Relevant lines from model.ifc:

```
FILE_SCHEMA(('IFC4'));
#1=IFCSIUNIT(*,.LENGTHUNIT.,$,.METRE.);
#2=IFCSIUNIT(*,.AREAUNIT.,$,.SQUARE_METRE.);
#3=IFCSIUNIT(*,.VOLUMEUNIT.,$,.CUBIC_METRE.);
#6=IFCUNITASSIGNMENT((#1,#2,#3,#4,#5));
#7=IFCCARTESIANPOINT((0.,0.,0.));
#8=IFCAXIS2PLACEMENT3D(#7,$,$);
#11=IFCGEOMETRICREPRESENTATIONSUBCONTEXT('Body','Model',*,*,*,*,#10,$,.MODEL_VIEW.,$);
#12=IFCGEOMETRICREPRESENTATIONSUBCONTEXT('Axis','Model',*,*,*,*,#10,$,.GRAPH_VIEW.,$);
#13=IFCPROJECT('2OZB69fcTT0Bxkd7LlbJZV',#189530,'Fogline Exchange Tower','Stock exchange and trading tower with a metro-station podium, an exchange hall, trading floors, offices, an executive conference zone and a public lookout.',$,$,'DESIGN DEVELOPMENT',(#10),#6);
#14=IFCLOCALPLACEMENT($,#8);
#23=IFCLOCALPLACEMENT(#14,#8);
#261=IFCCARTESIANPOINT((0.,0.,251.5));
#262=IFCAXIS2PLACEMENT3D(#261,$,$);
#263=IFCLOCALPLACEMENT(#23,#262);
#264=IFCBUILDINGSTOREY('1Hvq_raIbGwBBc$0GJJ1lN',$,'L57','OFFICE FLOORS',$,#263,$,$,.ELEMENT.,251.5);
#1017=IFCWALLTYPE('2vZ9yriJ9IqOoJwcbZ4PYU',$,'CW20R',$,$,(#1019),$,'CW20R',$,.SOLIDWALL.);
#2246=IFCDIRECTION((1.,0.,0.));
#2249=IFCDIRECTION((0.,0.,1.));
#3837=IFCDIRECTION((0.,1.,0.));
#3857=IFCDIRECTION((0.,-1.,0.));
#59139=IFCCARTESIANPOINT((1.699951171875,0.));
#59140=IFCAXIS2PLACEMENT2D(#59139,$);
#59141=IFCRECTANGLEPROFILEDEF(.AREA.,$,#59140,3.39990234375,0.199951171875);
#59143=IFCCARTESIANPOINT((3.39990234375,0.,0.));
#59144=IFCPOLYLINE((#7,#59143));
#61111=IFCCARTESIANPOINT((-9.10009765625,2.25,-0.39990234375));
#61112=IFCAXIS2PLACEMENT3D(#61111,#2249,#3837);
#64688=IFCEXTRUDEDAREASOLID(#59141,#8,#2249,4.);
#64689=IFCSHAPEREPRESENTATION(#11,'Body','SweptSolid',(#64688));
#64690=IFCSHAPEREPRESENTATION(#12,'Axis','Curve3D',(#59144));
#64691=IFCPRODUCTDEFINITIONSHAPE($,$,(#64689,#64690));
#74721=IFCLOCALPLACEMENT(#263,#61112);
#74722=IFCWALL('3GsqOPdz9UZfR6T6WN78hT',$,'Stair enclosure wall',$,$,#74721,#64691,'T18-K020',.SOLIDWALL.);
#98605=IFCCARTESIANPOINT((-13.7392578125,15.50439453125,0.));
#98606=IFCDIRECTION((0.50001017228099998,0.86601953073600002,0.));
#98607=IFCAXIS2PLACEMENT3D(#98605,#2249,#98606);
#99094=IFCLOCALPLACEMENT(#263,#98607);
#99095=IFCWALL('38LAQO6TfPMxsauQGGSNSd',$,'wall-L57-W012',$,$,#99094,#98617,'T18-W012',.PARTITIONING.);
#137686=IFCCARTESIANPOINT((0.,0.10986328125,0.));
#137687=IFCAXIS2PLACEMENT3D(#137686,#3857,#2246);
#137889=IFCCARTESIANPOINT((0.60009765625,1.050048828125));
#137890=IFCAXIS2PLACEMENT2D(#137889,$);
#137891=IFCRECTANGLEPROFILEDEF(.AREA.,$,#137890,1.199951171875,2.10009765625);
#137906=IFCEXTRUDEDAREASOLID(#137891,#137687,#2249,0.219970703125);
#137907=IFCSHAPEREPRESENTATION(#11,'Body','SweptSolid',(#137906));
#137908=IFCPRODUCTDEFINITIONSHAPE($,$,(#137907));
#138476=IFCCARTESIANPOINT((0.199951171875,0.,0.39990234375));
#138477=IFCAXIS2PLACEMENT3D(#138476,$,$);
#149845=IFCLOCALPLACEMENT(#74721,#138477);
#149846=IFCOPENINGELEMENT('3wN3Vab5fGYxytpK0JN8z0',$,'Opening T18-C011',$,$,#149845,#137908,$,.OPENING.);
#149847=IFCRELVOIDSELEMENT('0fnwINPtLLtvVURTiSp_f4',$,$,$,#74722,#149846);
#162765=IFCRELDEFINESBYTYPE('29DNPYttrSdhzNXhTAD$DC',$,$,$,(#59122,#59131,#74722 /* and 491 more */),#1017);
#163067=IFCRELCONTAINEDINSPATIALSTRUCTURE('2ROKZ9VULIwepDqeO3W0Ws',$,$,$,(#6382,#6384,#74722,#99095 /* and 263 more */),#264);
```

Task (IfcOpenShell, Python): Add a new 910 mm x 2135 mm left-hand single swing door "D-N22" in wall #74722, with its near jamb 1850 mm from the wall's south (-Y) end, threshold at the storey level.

```python
import numpy as np
import ifcopenshell
import ifcopenshell.api.feature
import ifcopenshell.api.geometry
import ifcopenshell.api.root
import ifcopenshell.api.spatial
import ifcopenshell.geom
import ifcopenshell.util.element
import ifcopenshell.util.placement
import ifcopenshell.util.representation
import ifcopenshell.util.shape
import ifcopenshell.util.unit

model = ifcopenshell.open("model.ifc")
unit_scale = ifcopenshell.util.unit.calculate_unit_scale(model)
settings = ifcopenshell.geom.settings()


def volume(element):
    """Net volume in cubic metres, openings subtracted."""
    shape = ifcopenshell.geom.create_shape(settings, element)
    return ifcopenshell.util.shape.get_volume(shape.geometry)


wall = model.by_id(74722)
storey = ifcopenshell.util.element.get_container(wall, ifc_class="IfcBuildingStorey")
context = ifcopenshell.util.representation.get_context(model, "Model", "Body", "MODEL_VIEW")
before = volume(wall)

width, height, from_end, sill = 0.91, 2.135, 1.85, 0.0  # metres

# The wall runs along its own X axis, and the end named is its -X end.
wall_shape = ifcopenshell.geom.create_shape(settings, wall)
x, y, z = ifcopenshell.util.shape.get_vertices(wall_shape.geometry).T
start = x.min() + from_end
face, thickness = float(y.min()), float(y.max() - y.min())
wall_matrix = ifcopenshell.util.placement.get_local_placement(wall.ObjectPlacement)
level = ifcopenshell.util.placement.get_local_placement(storey.ObjectPlacement)[2, 3]


def in_wall(x, y):
    """Placement at x, y metres in the wall's axes, at sill height."""
    matrix = wall_matrix.copy()
    matrix[:, 3] = wall_matrix @ np.array([x / unit_scale, y / unit_scale, 0.0, 1.0])
    matrix[2, 3] = level + sill / unit_scale
    return matrix


# Opening: a box that overshoots both wall faces by 50 mm.
opening = ifcopenshell.api.root.create_entity(model, ifc_class="IfcOpeningElement", predefined_type="OPENING")
box = ifcopenshell.api.geometry.add_wall_representation(
    model, context=context, length=width, height=height, thickness=thickness + 0.1
)
ifcopenshell.api.geometry.assign_representation(model, product=opening, representation=box)
ifcopenshell.api.geometry.edit_object_placement(model, product=opening, matrix=in_wall(start, face - 0.05), is_si=False)
ifcopenshell.api.feature.add_feature(model, feature=opening, element=wall)

door = ifcopenshell.api.root.create_entity(model, ifc_class="IfcDoor", name="D-N22", predefined_type="DOOR")
door.OverallWidth, door.OverallHeight = width / unit_scale, height / unit_scale
door.OperationType = "SINGLE_SWING_LEFT"
body = ifcopenshell.api.geometry.add_door_representation(
    model,
    context=context,
    overall_width=door.OverallWidth,
    overall_height=door.OverallHeight,
    operation_type="SINGLE_SWING_LEFT",
    lining_properties={"LiningDepth": thickness / unit_scale, "ThresholdDepth": thickness / unit_scale},
)
ifcopenshell.api.geometry.assign_representation(model, product=door, representation=body)
ifcopenshell.api.spatial.assign_container(model, products=[door], relating_structure=storey)
ifcopenshell.api.feature.add_filling(model, opening=opening, element=door)

# The lining spans the wall, so the door starts at the wall face.
ifcopenshell.api.geometry.edit_object_placement(model, product=door, matrix=in_wall(start, face), is_si=False)

after = volume(wall)

print(f"wall volume {before:.3f} -> {after:.3f} m3")

model.write("model_updated.ifc")
```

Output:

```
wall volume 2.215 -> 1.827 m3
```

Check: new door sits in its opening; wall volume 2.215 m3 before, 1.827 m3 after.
